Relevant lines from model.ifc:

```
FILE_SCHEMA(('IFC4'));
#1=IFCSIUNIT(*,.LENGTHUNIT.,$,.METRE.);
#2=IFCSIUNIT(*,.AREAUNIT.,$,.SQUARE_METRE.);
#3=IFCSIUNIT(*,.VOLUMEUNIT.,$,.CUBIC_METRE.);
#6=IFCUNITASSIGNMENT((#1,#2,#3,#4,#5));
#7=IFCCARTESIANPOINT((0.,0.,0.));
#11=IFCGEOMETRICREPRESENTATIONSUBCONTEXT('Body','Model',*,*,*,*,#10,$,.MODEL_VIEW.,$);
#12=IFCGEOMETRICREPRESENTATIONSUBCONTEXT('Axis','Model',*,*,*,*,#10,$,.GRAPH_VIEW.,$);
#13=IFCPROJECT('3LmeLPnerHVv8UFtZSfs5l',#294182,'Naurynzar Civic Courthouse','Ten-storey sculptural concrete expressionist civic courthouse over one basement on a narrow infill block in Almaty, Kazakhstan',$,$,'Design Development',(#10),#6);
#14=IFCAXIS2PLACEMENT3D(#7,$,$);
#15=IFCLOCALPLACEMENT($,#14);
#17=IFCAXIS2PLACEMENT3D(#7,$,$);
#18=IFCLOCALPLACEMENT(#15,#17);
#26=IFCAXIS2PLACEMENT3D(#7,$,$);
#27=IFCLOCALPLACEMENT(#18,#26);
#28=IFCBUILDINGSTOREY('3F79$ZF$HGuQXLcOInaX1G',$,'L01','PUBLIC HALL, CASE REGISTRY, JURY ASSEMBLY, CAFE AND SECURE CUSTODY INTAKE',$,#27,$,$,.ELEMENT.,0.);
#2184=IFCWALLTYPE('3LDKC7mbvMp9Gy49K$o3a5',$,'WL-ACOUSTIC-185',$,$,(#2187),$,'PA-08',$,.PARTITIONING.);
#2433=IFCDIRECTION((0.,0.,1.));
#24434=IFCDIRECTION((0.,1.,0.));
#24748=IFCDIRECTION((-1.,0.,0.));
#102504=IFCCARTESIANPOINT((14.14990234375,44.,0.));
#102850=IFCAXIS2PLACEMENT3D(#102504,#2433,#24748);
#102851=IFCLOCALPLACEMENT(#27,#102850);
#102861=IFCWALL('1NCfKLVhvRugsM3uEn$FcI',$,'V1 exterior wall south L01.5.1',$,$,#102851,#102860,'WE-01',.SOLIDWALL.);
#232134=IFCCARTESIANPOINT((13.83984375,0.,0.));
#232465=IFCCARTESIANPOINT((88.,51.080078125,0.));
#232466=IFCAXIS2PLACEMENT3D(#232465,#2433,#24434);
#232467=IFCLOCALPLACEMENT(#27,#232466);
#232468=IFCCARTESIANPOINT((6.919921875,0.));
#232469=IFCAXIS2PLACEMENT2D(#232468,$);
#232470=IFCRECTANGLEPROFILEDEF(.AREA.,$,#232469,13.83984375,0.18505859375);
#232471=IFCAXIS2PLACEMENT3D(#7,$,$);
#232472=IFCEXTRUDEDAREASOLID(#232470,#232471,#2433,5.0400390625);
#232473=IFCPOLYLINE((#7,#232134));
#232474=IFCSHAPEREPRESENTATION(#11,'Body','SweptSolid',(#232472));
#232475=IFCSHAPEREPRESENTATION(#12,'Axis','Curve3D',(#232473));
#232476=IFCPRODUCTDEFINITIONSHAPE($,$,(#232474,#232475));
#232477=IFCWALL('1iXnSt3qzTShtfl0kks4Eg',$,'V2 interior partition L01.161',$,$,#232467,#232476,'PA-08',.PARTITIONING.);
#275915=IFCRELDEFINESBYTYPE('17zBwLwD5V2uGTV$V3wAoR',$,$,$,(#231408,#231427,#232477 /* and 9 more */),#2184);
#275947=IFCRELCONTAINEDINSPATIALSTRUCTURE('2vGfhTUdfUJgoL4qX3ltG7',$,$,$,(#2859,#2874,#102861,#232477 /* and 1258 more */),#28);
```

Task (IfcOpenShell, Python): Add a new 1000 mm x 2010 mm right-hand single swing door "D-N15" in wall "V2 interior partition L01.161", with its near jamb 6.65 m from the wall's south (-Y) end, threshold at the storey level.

```python
import numpy as np
import ifcopenshell
import ifcopenshell.api.feature
import ifcopenshell.api.geometry
import ifcopenshell.api.root
import ifcopenshell.api.spatial
import ifcopenshell.geom
import ifcopenshell.util.element
import ifcopenshell.util.placement
import ifcopenshell.util.representation
import ifcopenshell.util.shape
import ifcopenshell.util.unit

model = ifcopenshell.open("model.ifc")
unit_scale = ifcopenshell.util.unit.calculate_unit_scale(model)
settings = ifcopenshell.geom.settings()


def volume(element):
    """Net volume in cubic metres, openings subtracted."""
    shape = ifcopenshell.geom.create_shape(settings, element)
    return ifcopenshell.util.shape.get_volume(shape.geometry)


wall = model.by_guid("1iXnSt3qzTShtfl0kks4Eg")
storey = ifcopenshell.util.element.get_container(wall, ifc_class="IfcBuildingStorey")
context = ifcopenshell.util.representation.get_context(model, "Model", "Body", "MODEL_VIEW")
before = volume(wall)

width, height, from_end, sill = 1, 2.01, 6.65, 0.0  # metres

# The wall runs along its own X axis, and the end named is its -X end.
wall_shape = ifcopenshell.geom.create_shape(settings, wall)
x, y, z = ifcopenshell.util.shape.get_vertices(wall_shape.geometry).T
start = x.min() + from_end
face, thickness = float(y.min()), float(y.max() - y.min())
wall_matrix = ifcopenshell.util.placement.get_local_placement(wall.ObjectPlacement)
level = ifcopenshell.util.placement.get_local_placement(storey.ObjectPlacement)[2, 3]


def in_wall(x, y):
    """Placement at x, y metres in the wall's axes, at sill height."""
    matrix = wall_matrix.copy()
    matrix[:, 3] = wall_matrix @ np.array([x / unit_scale, y / unit_scale, 0.0, 1.0])
    matrix[2, 3] = level + sill / unit_scale
    return matrix


# Opening: a box that overshoots both wall faces by 50 mm.
opening = ifcopenshell.api.root.create_entity(model, ifc_class="IfcOpeningElement", predefined_type="OPENING")
box = ifcopenshell.api.geometry.add_wall_representation(
    model, context=context, length=width, height=height, thickness=thickness + 0.1
)
ifcopenshell.api.geometry.assign_representation(model, product=opening, representation=box)
ifcopenshell.api.geometry.edit_object_placement(model, product=opening, matrix=in_wall(start, face - 0.05), is_si=False)
ifcopenshell.api.feature.add_feature(model, feature=opening, element=wall)

door = ifcopenshell.api.root.create_entity(model, ifc_class="IfcDoor", name="D-N15", predefined_type="DOOR")
door.OverallWidth, door.OverallHeight = width / unit_scale, height / unit_scale
door.OperationType = "SINGLE_SWING_RIGHT"
body = ifcopenshell.api.geometry.add_door_representation(
    model,
    context=context,
    overall_width=door.OverallWidth,
    overall_height=door.OverallHeight,
    operation_type="SINGLE_SWING_RIGHT",
    lining_properties={"LiningDepth": thickness / unit_scale, "ThresholdDepth": thickness / unit_scale},
)
ifcopenshell.api.geometry.assign_representation(model, product=door, representation=body)
ifcopenshell.api.spatial.assign_container(model, products=[door], relating_structure=storey)
ifcopenshell.api.feature.add_filling(model, opening=opening, element=door)

# The lining spans the wall, so the door starts at the wall face.
ifcopenshell.api.geometry.edit_object_placement(model, product=door, matrix=in_wall(start, face), is_si=False)

after = volume(wall)

print(f"wall volume {before:.3f} -> {after:.3f} m3")

model.write("model-out.ifc")
```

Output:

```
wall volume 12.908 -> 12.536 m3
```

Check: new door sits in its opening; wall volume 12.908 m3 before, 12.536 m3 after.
